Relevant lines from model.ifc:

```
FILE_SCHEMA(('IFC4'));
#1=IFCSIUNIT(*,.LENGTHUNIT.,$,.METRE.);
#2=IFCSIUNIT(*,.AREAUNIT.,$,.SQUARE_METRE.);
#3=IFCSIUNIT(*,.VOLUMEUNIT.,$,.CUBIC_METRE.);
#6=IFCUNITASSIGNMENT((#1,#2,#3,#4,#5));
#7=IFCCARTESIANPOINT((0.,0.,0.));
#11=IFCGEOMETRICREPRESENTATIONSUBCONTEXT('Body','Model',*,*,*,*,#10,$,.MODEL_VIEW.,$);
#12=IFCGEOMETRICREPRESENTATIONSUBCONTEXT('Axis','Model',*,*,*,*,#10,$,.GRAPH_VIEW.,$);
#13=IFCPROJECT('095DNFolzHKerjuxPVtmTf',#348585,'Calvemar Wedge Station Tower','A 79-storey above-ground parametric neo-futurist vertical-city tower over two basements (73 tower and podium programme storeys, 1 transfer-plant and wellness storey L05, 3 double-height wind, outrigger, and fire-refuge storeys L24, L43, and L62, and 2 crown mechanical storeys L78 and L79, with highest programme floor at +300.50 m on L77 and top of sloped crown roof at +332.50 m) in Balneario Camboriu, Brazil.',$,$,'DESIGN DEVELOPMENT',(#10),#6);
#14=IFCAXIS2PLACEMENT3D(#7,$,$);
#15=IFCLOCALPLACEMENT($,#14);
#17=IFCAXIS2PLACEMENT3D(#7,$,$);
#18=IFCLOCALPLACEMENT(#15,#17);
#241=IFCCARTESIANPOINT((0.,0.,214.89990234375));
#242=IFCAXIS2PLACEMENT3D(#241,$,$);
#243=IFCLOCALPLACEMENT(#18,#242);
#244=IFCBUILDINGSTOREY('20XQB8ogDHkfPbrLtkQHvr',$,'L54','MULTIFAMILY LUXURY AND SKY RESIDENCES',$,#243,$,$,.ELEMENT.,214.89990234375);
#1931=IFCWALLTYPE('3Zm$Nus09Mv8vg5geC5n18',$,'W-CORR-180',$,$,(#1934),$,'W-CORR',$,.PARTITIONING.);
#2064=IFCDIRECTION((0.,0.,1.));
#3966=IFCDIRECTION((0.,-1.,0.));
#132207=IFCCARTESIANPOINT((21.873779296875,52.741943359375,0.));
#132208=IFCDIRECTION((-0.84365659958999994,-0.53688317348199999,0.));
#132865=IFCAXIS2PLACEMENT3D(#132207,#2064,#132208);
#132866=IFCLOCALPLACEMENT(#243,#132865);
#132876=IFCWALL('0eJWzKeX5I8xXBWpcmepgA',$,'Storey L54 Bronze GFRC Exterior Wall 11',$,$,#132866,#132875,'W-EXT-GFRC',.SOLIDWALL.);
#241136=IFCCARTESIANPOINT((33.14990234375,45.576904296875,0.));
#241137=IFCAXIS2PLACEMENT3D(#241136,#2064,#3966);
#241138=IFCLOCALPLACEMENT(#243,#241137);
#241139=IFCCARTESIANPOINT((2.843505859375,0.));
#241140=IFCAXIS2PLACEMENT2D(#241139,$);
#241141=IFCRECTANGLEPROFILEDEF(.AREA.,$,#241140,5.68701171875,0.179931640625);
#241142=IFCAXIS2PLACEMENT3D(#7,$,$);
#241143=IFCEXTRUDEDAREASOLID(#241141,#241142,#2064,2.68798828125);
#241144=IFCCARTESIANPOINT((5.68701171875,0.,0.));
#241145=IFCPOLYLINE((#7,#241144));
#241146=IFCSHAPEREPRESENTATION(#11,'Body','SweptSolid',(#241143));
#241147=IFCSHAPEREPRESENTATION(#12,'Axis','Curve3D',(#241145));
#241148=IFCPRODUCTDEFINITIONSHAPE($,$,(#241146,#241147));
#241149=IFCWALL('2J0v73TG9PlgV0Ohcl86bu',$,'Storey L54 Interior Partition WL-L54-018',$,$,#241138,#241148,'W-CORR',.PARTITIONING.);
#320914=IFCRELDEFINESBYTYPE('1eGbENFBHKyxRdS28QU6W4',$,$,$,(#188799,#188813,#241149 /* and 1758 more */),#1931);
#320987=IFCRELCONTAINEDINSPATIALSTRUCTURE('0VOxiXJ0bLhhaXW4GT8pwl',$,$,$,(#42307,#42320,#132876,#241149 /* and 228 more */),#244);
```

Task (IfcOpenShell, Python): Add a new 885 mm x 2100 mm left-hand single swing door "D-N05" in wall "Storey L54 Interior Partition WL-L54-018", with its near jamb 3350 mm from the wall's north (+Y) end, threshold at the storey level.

```python
import numpy as np
import ifcopenshell
import ifcopenshell.api.feature
import ifcopenshell.api.geometry
import ifcopenshell.api.root
import ifcopenshell.api.spatial
import ifcopenshell.geom
import ifcopenshell.util.element
import ifcopenshell.util.placement
import ifcopenshell.util.representation
import ifcopenshell.util.shape
import ifcopenshell.util.unit

model = ifcopenshell.open("model.ifc")
unit_scale = ifcopenshell.util.unit.calculate_unit_scale(model)
settings = ifcopenshell.geom.settings()


def volume(element):
    """Net volume in cubic metres, openings subtracted."""
    shape = ifcopenshell.geom.create_shape(settings, element)
    return ifcopenshell.util.shape.get_volume(shape.geometry)


wall = model.by_id(241149)
storey = ifcopenshell.util.element.get_container(wall, ifc_class="IfcBuildingStorey")
context = ifcopenshell.util.representation.get_context(model, "Model", "Body", "MODEL_VIEW")
before = volume(wall)

width, height, from_end, sill = 0.885, 2.1, 3.35, 0.0  # metres

# The wall runs along its own X axis, and the end named is its -X end.
wall_shape = ifcopenshell.geom.create_shape(settings, wall)
x, y, z = ifcopenshell.util.shape.get_vertices(wall_shape.geometry).T
start = x.min() + from_end
face, thickness = float(y.min()), float(y.max() - y.min())
wall_matrix = ifcopenshell.util.placement.get_local_placement(wall.ObjectPlacement)
level = ifcopenshell.util.placement.get_local_placement(storey.ObjectPlacement)[2, 3]


def in_wall(x, y):
    """Placement at x, y metres in the wall's axes, at sill height."""
    matrix = wall_matrix.copy()
    matrix[:, 3] = wall_matrix @ np.array([x / unit_scale, y / unit_scale, 0.0, 1.0])
    matrix[2, 3] = level + sill / unit_scale
    return matrix


# Opening: a box that overshoots both wall faces by 50 mm.
opening = ifcopenshell.api.root.create_entity(model, ifc_class="IfcOpeningElement", predefined_type="OPENING")
box = ifcopenshell.api.geometry.add_wall_representation(
    model, context=context, length=width, height=height, thickness=thickness + 0.1
)
ifcopenshell.api.geometry.assign_representation(model, product=opening, representation=box)
ifcopenshell.api.geometry.edit_object_placement(model, product=opening, matrix=in_wall(start, face - 0.05), is_si=False)
ifcopenshell.api.feature.add_feature(model, feature=opening, element=wall)

door = ifcopenshell.api.root.create_entity(model, ifc_class="IfcDoor", name="D-N05", predefined_type="DOOR")
door.OverallWidth, door.OverallHeight = width / unit_scale, height / unit_scale
door.OperationType = "SINGLE_SWING_LEFT"
body = ifcopenshell.api.geometry.add_door_representation(
    model,
    context=context,
    overall_width=door.OverallWidth,
    overall_height=door.OverallHeight,
    operation_type="SINGLE_SWING_LEFT",
    lining_properties={"LiningDepth": thickness / unit_scale, "ThresholdDepth": thickness / unit_scale},
)
ifcopenshell.api.geometry.assign_representation(model, product=door, representation=body)
ifcopenshell.api.spatial.assign_container(model, products=[door], relating_structure=storey)
ifcopenshell.api.feature.add_filling(model, opening=opening, element=door)

# The lining spans the wall, so the door starts at the wall face.
ifcopenshell.api.geometry.edit_object_placement(model, product=door, matrix=in_wall(start, face), is_si=False)

after = volume(wall)

print(f"wall volume {before:.3f} -> {after:.3f} m3")

model.write("model_v2.ifc")
```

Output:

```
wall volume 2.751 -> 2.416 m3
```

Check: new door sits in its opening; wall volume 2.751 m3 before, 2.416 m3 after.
